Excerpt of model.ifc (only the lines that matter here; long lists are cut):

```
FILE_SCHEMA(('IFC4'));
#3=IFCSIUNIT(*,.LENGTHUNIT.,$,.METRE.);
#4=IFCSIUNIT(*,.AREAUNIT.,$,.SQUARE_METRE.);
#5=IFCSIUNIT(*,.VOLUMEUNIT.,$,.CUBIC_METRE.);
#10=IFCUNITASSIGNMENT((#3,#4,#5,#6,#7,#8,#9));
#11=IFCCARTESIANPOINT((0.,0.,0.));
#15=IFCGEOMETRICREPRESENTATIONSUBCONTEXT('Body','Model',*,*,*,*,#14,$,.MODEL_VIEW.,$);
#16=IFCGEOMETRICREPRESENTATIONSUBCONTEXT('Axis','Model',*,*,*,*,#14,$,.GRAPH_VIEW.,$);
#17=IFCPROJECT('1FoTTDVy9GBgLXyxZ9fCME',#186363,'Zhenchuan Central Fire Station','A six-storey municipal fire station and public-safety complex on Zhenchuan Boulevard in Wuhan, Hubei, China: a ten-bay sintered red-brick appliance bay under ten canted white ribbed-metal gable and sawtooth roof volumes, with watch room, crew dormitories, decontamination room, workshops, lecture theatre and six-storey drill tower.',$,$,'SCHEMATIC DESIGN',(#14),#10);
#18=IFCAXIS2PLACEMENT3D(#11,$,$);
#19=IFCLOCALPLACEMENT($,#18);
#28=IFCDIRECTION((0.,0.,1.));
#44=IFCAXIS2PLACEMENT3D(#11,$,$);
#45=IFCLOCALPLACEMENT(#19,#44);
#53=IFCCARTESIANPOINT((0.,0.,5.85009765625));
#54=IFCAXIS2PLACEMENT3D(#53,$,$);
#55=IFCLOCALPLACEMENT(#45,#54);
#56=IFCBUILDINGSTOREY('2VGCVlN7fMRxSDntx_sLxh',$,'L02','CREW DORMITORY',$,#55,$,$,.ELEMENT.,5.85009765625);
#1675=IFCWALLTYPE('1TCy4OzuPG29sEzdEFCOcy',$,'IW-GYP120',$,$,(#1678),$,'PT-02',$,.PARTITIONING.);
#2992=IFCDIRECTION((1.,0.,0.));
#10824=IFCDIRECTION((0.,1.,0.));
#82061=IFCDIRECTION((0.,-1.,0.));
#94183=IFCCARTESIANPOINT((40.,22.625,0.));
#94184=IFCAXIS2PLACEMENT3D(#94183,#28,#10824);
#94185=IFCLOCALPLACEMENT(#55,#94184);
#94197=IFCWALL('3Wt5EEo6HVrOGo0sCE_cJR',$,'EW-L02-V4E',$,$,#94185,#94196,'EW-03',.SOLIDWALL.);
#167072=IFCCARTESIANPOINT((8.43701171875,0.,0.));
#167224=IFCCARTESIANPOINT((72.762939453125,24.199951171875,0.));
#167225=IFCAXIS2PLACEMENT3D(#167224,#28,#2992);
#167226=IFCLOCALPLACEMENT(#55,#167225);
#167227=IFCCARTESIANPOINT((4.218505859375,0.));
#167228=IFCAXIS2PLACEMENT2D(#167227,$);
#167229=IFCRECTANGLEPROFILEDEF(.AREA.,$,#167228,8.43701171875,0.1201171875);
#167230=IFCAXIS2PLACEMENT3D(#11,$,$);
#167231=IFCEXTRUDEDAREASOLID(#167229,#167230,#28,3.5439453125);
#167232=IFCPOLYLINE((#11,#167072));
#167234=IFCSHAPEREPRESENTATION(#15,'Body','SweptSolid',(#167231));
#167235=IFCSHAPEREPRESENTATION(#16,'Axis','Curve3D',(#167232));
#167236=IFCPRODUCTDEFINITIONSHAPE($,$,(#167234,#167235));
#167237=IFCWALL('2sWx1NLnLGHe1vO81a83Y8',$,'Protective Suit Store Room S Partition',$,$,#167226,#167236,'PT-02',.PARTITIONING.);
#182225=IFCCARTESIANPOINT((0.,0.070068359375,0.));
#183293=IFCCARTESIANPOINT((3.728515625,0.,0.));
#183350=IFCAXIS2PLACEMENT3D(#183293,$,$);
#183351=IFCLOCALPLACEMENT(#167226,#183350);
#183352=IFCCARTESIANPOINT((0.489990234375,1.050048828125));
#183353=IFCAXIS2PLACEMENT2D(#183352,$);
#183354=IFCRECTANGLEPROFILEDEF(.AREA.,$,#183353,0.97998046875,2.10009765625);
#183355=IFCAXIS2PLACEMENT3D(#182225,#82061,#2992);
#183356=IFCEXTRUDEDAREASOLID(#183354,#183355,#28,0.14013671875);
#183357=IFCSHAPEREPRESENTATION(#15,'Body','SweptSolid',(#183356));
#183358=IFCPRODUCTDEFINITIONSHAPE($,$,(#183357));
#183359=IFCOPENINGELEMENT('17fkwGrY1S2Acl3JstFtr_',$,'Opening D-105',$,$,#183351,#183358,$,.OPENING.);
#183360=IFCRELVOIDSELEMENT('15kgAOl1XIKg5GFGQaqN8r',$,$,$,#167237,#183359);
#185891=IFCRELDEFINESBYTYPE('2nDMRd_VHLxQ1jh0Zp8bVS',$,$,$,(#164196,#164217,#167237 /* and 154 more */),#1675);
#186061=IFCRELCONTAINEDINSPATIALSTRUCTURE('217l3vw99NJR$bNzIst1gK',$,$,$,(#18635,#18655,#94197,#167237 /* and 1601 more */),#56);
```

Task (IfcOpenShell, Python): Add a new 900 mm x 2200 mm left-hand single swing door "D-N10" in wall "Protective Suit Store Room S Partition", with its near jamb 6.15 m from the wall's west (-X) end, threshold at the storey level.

```python
import numpy as np
import ifcopenshell
import ifcopenshell.api.feature
import ifcopenshell.api.geometry
import ifcopenshell.api.root
import ifcopenshell.api.spatial
import ifcopenshell.geom
import ifcopenshell.util.element
import ifcopenshell.util.placement
import ifcopenshell.util.representation
import ifcopenshell.util.shape
import ifcopenshell.util.unit

model = ifcopenshell.open("model.ifc")
unit_scale = ifcopenshell.util.unit.calculate_unit_scale(model)
settings = ifcopenshell.geom.settings()


def volume(element):
    """Net volume in cubic metres, openings subtracted."""
    shape = ifcopenshell.geom.create_shape(settings, element)
    return ifcopenshell.util.shape.get_volume(shape.geometry)


wall = model.by_id(167237)
storey = ifcopenshell.util.element.get_container(wall, ifc_class="IfcBuildingStorey")
context = ifcopenshell.util.representation.get_context(model, "Model", "Body", "MODEL_VIEW")
before = volume(wall)

width, height, from_end, sill = 0.9, 2.2, 6.15, 0.0  # metres

# The wall runs along its own X axis, and the end named is its -X end.
wall_shape = ifcopenshell.geom.create_shape(settings, wall)
x, y, z = ifcopenshell.util.shape.get_vertices(wall_shape.geometry).T
start = x.min() + from_end
face, thickness = float(y.min()), float(y.max() - y.min())
wall_matrix = ifcopenshell.util.placement.get_local_placement(wall.ObjectPlacement)
level = ifcopenshell.util.placement.get_local_placement(storey.ObjectPlacement)[2, 3]


def in_wall(x, y):
    """Placement at x, y metres in the wall's axes, at sill height."""
    matrix = wall_matrix.copy()
    matrix[:, 3] = wall_matrix @ np.array([x / unit_scale, y / unit_scale, 0.0, 1.0])
    matrix[2, 3] = level + sill / unit_scale
    return matrix


# Opening: a box that overshoots both wall faces by 50 mm.
opening = ifcopenshell.api.root.create_entity(model, ifc_class="IfcOpeningElement", predefined_type="OPENING")
box = ifcopenshell.api.geometry.add_wall_representation(
    model, context=context, length=width, height=height, thickness=thickness + 0.1
)
ifcopenshell.api.geometry.assign_representation(model, product=opening, representation=box)
ifcopenshell.api.geometry.edit_object_placement(model, product=opening, matrix=in_wall(start, face - 0.05), is_si=False)
ifcopenshell.api.feature.add_feature(model, feature=opening, element=wall)

door = ifcopenshell.api.root.create_entity(model, ifc_class="IfcDoor", name="D-N10", predefined_type="DOOR")
door.OverallWidth, door.OverallHeight = width / unit_scale, height / unit_scale
door.OperationType = "SINGLE_SWING_LEFT"
body = ifcopenshell.api.geometry.add_door_representation(
    model,
    context=context,
    overall_width=door.OverallWidth,
    overall_height=door.OverallHeight,
    operation_type="SINGLE_SWING_LEFT",
    lining_properties={"LiningDepth": thickness / unit_scale, "ThresholdDepth": thickness / unit_scale},
)
ifcopenshell.api.geometry.assign_representation(model, product=door, representation=body)
ifcopenshell.api.spatial.assign_container(model, products=[door], relating_structure=storey)
ifcopenshell.api.feature.add_filling(model, opening=opening, element=door)

# The lining spans the wall, so the door starts at the wall face.
ifcopenshell.api.geometry.edit_object_placement(model, product=door, matrix=in_wall(start, face), is_si=False)

after = volume(wall)

print(f"wall volume {before:.3f} -> {after:.3f} m3")

model.write("model_edited.ifc")
```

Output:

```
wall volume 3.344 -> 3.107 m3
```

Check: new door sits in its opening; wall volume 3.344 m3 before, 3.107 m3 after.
